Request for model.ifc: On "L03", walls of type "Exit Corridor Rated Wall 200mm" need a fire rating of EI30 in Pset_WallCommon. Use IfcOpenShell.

First a look at what the model holds.

```python
import ifcopenshell
import ifcopenshell.util.element

model = ifcopenshell.open("model.ifc")
print(model.schema)
storey = next(s for s in model.by_type("IfcBuildingStorey") if s.Name == "L03")
walls = [e for e in ifcopenshell.util.element.get_decomposition(storey) if e.is_a("IfcWall")]
seen = {}
for e in walls:
    element_type = ifcopenshell.util.element.get_type(e)
    key = (element_type.Name if element_type != e and element_type else None, ifcopenshell.util.element.get_pset(e, "Pset_WallCommon", "FireRating"))
    seen[key] = seen.get(key, 0) + 1
for (name, value), count in sorted(seen.items(), key=str):
    print(count, "x", name, "|", value)
```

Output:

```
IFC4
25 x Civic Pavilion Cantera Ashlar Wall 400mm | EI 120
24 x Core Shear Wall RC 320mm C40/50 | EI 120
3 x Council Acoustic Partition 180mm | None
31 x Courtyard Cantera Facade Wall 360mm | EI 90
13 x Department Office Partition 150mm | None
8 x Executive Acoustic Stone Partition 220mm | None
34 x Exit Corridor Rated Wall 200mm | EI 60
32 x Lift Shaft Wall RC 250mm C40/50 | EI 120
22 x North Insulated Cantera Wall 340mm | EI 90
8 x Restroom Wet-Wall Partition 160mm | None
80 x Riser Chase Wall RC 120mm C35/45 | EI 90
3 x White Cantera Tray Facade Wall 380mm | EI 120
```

```python
import ifcopenshell
import ifcopenshell.api.pset
import ifcopenshell.util.element

model = ifcopenshell.open("model.ifc")

storey = next(s for s in model.by_type("IfcBuildingStorey") if s.Name == "L03")
walls = [e for e in ifcopenshell.util.element.get_decomposition(storey) if e.is_a("IfcWall")]

count = 0
for e in walls:
    element_type = ifcopenshell.util.element.get_type(e)
    if element_type in (None, e) or element_type.Name != "Exit Corridor Rated Wall 200mm":
        continue
    # add_pset returns the element's existing set when there is one.
    pset = ifcopenshell.api.pset.add_pset(model, product=e, name="Pset_WallCommon")
    ifcopenshell.api.pset.edit_pset(model, pset=pset, properties={"FireRating": "EI30"})
    count += 1

print(count, "walls updated")

model.write("model_v2.ifc")
```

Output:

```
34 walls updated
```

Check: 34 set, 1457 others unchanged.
